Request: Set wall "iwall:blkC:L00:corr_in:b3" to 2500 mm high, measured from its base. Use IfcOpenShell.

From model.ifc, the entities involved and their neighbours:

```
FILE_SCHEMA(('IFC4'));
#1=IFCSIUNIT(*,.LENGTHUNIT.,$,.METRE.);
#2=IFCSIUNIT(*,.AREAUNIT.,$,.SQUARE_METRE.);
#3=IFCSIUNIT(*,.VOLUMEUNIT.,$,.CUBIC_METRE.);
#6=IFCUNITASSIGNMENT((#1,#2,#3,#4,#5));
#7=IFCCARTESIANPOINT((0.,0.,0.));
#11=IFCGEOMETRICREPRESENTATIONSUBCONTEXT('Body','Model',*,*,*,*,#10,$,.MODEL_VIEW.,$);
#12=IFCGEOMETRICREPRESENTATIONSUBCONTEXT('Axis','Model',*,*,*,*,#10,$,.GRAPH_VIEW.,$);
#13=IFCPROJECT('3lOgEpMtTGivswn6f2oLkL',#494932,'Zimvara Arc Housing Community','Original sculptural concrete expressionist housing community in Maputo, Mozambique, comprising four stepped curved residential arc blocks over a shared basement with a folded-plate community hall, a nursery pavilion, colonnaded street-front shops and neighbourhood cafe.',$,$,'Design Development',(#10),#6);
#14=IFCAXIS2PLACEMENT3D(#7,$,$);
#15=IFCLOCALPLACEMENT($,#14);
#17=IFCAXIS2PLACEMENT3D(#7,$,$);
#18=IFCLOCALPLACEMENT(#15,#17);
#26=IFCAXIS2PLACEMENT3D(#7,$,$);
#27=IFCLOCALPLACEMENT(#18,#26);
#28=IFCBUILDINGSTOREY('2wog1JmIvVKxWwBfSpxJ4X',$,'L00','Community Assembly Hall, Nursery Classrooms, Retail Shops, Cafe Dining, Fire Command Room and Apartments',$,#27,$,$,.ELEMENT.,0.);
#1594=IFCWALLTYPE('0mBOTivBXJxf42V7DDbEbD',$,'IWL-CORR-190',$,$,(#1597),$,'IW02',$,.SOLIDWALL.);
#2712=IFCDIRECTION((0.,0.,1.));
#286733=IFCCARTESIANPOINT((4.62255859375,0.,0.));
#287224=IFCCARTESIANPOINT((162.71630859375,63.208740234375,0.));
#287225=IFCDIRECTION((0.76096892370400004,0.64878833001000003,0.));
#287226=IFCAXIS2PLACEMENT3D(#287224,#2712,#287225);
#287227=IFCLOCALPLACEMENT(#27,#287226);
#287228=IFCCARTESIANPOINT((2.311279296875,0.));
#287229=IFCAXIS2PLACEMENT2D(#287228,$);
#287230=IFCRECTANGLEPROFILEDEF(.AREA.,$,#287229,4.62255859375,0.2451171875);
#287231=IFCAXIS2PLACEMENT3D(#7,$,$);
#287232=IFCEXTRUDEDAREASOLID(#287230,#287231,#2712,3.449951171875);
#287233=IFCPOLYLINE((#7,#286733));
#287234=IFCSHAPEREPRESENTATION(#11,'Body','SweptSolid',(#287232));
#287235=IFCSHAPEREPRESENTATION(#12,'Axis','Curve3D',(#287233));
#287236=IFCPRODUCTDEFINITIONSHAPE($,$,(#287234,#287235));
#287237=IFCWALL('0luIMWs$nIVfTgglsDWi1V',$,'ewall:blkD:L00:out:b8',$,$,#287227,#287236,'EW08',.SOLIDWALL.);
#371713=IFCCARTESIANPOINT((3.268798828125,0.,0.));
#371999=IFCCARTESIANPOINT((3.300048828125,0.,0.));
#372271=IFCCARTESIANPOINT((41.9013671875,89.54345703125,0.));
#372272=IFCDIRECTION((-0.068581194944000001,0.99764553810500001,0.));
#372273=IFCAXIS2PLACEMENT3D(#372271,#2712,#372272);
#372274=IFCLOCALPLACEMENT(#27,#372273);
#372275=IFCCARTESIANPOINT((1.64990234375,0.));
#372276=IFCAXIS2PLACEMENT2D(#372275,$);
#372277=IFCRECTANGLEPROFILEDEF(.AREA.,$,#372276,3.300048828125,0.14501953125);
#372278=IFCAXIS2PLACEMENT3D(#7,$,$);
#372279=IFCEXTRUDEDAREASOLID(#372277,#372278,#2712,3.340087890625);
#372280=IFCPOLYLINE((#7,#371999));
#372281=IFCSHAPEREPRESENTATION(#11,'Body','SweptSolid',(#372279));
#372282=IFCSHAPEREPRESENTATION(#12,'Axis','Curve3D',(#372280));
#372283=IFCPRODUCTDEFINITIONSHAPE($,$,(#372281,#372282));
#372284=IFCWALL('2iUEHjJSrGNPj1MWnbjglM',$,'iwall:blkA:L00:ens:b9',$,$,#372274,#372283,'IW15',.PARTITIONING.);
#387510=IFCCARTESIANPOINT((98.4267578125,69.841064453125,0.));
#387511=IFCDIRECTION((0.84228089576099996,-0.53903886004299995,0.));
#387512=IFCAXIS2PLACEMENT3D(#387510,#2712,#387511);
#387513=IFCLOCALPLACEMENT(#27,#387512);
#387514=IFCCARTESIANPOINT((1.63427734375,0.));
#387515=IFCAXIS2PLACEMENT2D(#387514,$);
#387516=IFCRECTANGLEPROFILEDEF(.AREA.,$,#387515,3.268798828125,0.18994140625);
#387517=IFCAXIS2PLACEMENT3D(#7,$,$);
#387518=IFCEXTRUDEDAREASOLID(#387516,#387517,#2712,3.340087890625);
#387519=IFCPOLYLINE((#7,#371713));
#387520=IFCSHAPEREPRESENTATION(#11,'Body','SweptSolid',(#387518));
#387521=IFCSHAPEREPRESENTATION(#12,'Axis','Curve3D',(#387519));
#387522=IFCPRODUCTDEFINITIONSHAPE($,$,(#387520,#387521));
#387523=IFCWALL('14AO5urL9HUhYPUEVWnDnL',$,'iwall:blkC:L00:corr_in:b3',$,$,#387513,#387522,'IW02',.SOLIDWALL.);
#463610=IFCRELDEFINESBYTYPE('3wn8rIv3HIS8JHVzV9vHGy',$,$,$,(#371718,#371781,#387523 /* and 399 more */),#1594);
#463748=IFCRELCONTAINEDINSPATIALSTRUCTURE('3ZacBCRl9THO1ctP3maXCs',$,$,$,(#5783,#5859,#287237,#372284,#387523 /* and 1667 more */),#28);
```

```python
import ifcopenshell
import ifcopenshell.geom
import ifcopenshell.util.representation
import ifcopenshell.util.shape
import ifcopenshell.util.unit

model = ifcopenshell.open("model.ifc")
unit_scale = ifcopenshell.util.unit.calculate_unit_scale(model)
settings = ifcopenshell.geom.settings()


def volume(element):
    """Net volume in cubic metres, openings subtracted."""
    shape = ifcopenshell.geom.create_shape(settings, element)
    return ifcopenshell.util.shape.get_volume(shape.geometry)


wall = model.by_id(387523)
before = volume(wall)

body = ifcopenshell.util.representation.get_representation(wall, "Model", "Body")
solid = body.Items[0]
old_height = solid.Depth
solid.Depth = 2.5 / unit_scale
after = volume(wall)

print(f"height {old_height:g} -> {solid.Depth:g}, volume {before:.3f} -> {after:.3f} m3")

model.write("model_rev.ifc")
```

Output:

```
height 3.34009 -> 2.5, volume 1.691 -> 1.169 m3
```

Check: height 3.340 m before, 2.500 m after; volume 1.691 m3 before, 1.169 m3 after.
